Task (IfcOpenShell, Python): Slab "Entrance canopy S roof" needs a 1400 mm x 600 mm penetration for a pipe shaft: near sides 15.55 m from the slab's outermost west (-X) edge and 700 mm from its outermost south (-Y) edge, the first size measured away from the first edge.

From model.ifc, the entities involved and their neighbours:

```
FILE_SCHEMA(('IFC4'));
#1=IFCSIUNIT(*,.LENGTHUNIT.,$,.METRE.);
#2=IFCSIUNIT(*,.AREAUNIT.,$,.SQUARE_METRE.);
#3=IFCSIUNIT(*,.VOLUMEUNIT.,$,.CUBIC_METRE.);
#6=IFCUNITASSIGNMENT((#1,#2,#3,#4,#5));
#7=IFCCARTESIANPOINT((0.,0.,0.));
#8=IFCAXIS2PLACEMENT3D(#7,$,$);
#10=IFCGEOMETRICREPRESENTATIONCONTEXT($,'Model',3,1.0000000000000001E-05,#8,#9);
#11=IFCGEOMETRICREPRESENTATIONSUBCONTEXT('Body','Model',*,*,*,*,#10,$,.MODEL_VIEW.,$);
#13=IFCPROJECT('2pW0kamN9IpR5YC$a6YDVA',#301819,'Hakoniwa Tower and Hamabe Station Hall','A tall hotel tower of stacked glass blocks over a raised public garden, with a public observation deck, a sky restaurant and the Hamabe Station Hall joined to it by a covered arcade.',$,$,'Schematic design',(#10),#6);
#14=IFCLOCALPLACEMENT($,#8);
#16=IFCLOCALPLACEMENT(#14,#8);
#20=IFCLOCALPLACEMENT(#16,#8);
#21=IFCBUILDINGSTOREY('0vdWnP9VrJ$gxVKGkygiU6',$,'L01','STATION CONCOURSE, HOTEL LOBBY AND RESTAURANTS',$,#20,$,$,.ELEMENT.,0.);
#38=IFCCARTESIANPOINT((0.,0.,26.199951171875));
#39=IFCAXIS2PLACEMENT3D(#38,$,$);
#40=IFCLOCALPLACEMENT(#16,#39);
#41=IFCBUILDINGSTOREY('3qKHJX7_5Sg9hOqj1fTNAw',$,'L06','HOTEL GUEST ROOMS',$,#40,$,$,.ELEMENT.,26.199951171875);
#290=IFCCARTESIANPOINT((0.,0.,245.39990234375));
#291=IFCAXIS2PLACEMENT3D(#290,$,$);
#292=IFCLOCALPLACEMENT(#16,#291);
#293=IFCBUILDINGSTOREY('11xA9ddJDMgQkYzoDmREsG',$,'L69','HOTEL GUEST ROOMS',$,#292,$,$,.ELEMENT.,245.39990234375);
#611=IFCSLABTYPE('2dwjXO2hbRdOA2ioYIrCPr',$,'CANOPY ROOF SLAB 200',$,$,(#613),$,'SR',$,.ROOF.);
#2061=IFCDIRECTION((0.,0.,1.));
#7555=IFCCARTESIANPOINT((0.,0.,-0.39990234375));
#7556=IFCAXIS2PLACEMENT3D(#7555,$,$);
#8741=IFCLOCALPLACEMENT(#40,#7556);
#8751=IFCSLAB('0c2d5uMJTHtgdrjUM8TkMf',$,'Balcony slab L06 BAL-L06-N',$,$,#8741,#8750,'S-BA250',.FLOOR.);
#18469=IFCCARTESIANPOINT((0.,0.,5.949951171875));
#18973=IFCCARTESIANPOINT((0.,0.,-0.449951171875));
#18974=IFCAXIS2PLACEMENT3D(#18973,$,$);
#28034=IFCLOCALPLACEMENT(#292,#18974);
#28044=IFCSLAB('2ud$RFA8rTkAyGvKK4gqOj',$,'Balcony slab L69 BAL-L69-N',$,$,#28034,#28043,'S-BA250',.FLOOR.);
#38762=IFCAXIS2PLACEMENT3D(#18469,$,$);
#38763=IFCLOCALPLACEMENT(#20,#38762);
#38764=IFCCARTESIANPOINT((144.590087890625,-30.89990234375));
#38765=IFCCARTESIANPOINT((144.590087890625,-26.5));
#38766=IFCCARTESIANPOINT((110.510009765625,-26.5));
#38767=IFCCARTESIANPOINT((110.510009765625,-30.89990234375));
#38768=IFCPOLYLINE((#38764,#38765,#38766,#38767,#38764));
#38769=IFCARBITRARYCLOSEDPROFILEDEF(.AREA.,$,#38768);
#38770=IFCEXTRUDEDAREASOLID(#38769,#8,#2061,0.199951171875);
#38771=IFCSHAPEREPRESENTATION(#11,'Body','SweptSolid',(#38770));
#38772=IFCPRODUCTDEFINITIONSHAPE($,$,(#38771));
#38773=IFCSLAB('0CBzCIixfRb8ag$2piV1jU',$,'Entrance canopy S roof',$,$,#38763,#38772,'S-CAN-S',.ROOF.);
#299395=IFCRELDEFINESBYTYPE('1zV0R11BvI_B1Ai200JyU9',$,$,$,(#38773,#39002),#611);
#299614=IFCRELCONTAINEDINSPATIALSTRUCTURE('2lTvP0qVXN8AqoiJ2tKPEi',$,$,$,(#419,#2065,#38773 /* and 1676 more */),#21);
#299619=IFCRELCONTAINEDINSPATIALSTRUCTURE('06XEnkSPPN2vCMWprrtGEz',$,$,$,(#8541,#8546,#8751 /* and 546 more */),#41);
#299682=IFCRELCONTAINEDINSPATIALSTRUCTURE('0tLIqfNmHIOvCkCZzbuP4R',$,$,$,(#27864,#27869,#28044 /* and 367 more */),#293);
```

```python
import numpy as np
import ifcopenshell
import ifcopenshell.api.feature
import ifcopenshell.api.geometry
import ifcopenshell.api.root
import ifcopenshell.geom
import ifcopenshell.util.placement
import ifcopenshell.util.representation
import ifcopenshell.util.shape
import ifcopenshell.util.unit

model = ifcopenshell.open("model.ifc")
unit_scale = ifcopenshell.util.unit.calculate_unit_scale(model)
settings = ifcopenshell.geom.settings()


def volume(element):
    """Net volume in cubic metres, openings subtracted."""
    shape = ifcopenshell.geom.create_shape(settings, element)
    return ifcopenshell.util.shape.get_volume(shape.geometry)


slab = model.by_guid("0CBzCIixfRb8ag$2piV1jU")
before = volume(slab)

# Extent in the slab's own axes, in metres. The edges named are its -X and -Y sides.
slab_shape = ifcopenshell.geom.create_shape(settings, slab)
vertices = ifcopenshell.util.shape.get_vertices(slab_shape.geometry)
x_min, y_min, bottom = vertices.min(axis=0)
top = vertices[:, 2].max()

opening = ifcopenshell.api.root.create_entity(model, ifc_class="IfcOpeningElement", name="Pipe shaft opening", predefined_type="OPENING")
context = ifcopenshell.util.representation.get_context(model, "Model", "Body", "MODEL_VIEW")
width, depth = 1.4, 0.6
outline = [(0.0, 0.0), (width, 0.0), (width, depth), (0.0, depth), (0.0, 0.0)]
# Overshoot both faces by 50 mm so the cut is clean.
shape = ifcopenshell.api.geometry.add_slab_representation(
    model, context=context, depth=top - bottom + 0.1, polyline=outline
)
ifcopenshell.api.geometry.assign_representation(model, product=opening, representation=shape)

matrix = ifcopenshell.util.placement.get_local_placement(slab.ObjectPlacement)
matrix[:, 3] = matrix @ np.append(np.array([x_min + 15.55, y_min + 0.7, bottom - 0.05]) / unit_scale, 1.0)
ifcopenshell.api.geometry.edit_object_placement(model, product=opening, matrix=matrix, is_si=False)
ifcopenshell.api.feature.add_feature(model, feature=opening, element=slab)

after = volume(slab)

print(f"slab volume {before:.3f} -> {after:.3f} m3")

model.write("model_v2.ifc")
```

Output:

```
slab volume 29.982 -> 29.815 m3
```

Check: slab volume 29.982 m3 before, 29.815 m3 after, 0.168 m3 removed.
